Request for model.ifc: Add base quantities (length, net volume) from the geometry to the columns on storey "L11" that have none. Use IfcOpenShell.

First a look at what the model holds.

```python
import ifcopenshell
import ifcopenshell.util.element
import ifcopenshell.util.unit

model = ifcopenshell.open("model.ifc")
print(model.schema)
for unit_type in ("LENGTHUNIT", "AREAUNIT", "VOLUMEUNIT"):
    print(unit_type, ifcopenshell.util.unit.calculate_unit_scale(model, unit_type))
storey = next(s for s in model.by_type("IfcBuildingStorey") if s.Name == "L11")
columns = [e for e in ifcopenshell.util.element.get_decomposition(storey) if e.is_a("IfcColumn")]
for e in sorted(columns, key=lambda e: e.id()):
    print(e.id(), e.is_a(), e.Name, list(ifcopenshell.util.element.get_psets(e, qtos_only=True)), sep=" | ")
```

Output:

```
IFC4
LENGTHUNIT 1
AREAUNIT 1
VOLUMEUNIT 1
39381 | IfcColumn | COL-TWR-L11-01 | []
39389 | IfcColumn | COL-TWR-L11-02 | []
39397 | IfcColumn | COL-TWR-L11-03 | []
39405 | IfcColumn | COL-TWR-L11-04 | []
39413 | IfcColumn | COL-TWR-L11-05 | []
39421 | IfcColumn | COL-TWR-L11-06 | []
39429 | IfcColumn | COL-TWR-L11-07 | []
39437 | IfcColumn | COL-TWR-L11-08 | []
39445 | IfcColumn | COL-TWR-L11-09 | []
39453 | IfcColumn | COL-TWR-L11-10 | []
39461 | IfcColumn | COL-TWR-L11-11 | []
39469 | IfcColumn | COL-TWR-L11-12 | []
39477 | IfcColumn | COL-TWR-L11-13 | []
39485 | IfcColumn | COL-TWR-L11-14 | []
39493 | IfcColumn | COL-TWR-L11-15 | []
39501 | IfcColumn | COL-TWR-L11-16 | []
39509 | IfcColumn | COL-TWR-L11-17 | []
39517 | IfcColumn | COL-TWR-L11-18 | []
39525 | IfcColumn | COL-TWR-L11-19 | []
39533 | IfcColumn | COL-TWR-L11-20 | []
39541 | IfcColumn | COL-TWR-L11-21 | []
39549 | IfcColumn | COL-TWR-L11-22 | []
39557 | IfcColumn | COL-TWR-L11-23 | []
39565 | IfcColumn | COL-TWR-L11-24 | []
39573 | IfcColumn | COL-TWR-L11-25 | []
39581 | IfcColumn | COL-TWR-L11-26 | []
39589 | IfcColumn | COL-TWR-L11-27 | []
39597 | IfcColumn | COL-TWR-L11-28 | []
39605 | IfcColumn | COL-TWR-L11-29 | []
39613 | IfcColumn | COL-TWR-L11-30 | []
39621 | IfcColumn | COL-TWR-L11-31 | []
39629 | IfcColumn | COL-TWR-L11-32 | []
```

```python
import ifcopenshell
import ifcopenshell.api.pset
import ifcopenshell.geom
import ifcopenshell.util.element
import ifcopenshell.util.shape
import ifcopenshell.util.unit

model = ifcopenshell.open("model.ifc")
unit_scale = ifcopenshell.util.unit.calculate_unit_scale(model)
volume_scale = ifcopenshell.util.unit.calculate_unit_scale(model, "VOLUMEUNIT")
settings = ifcopenshell.geom.settings()

storey = next(s for s in model.by_type("IfcBuildingStorey") if s.Name == "L11")
columns = [e for e in ifcopenshell.util.element.get_decomposition(storey) if e.is_a("IfcColumn")]

for e in sorted(columns, key=lambda e: e.id()):
    if ifcopenshell.util.element.get_psets(e, qtos_only=True, should_inherit=False):
        continue
    # Geometry comes back in metres, in the element's own axes.
    shape = ifcopenshell.geom.create_shape(settings, e)
    values = {
        "Length": ifcopenshell.util.shape.get_z(shape.geometry) / unit_scale,
        "NetVolume": ifcopenshell.util.shape.get_volume(shape.geometry) / volume_scale,
    }
    qto = ifcopenshell.api.pset.add_qto(model, product=e, name="Qto_ColumnBaseQuantities")
    ifcopenshell.api.pset.edit_qto(model, qto=qto, properties=values)
    print(e.id(), {k: round(v, 3) for k, v in values.items()})

model.write("model_rev.ifc")
```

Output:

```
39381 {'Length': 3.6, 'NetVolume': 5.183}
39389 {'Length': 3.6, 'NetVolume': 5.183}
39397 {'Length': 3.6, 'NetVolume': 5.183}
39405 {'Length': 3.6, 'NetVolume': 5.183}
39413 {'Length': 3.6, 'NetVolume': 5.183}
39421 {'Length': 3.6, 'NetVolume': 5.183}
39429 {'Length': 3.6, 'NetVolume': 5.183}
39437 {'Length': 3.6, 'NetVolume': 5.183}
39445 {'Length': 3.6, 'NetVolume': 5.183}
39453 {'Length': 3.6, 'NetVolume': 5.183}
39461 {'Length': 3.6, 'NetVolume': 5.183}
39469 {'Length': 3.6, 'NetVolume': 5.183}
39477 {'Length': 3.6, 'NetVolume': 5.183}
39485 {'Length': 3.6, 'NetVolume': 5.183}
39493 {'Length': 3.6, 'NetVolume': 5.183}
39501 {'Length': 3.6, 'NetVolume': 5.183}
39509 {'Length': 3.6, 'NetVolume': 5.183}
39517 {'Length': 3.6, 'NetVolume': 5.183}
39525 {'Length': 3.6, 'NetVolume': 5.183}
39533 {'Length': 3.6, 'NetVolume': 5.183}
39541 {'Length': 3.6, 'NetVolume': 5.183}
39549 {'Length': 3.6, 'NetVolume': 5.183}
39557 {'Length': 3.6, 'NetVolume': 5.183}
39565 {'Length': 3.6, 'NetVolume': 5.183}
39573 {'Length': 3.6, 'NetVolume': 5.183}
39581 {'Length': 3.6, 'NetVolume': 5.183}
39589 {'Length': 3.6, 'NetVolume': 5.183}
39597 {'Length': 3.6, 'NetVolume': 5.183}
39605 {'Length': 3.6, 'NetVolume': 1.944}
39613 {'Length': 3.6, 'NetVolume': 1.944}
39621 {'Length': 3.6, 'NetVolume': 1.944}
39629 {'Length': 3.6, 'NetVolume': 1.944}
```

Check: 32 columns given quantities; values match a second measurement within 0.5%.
